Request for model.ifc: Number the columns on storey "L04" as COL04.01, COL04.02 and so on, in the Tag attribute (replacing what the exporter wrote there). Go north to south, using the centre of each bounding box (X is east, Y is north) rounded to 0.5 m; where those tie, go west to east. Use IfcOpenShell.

First a look at what the model holds.

```python
import ifcopenshell
import ifcopenshell.util.element
import ifcopenshell.util.placement

model = ifcopenshell.open("model.ifc")
print(model.schema)
storey = next(s for s in model.by_type("IfcBuildingStorey") if s.Name == "L04")
columns = [e for e in ifcopenshell.util.element.get_decomposition(storey) if e.is_a("IfcColumn")]
for e in sorted(columns, key=lambda e: e.id()):
    origin = ifcopenshell.util.placement.get_local_placement(e.ObjectPlacement)[:3, 3]
    print(e.id(), e.Tag, e.Name, origin.round(2) + 0.0, sep=" | ")
```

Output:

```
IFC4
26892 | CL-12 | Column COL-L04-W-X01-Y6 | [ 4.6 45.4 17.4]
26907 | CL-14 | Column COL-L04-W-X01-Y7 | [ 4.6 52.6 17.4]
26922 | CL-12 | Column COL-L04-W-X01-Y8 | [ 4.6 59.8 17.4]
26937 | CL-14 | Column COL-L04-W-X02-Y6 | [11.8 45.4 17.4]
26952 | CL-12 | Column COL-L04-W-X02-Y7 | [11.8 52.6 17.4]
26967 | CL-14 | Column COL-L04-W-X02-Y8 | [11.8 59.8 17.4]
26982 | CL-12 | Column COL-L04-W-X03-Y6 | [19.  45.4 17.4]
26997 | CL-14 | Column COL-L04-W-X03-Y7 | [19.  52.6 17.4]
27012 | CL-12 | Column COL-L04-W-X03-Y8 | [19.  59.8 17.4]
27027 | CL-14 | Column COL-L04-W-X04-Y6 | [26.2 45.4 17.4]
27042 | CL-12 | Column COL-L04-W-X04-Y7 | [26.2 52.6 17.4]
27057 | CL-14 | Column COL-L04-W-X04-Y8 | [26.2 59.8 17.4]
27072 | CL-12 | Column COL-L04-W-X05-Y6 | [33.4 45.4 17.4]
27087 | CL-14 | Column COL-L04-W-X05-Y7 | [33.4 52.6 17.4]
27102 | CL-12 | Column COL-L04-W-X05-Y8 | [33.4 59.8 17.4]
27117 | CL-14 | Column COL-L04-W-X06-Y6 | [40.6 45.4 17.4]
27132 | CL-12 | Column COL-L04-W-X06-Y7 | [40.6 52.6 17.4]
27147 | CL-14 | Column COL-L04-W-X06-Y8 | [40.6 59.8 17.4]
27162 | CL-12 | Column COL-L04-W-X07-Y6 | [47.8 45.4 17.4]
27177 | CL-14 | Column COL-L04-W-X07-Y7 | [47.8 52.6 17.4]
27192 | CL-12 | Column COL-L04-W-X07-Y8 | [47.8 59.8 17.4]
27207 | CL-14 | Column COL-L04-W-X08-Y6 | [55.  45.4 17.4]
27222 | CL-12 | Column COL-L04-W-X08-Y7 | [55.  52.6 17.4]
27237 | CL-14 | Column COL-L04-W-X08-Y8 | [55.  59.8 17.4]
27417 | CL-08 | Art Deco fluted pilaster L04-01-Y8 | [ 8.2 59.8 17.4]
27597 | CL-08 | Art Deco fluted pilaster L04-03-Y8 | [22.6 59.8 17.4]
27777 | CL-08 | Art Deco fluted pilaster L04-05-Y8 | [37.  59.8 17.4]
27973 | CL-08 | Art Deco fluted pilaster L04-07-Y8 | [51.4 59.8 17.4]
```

```python
import ifcopenshell
import ifcopenshell.geom
import ifcopenshell.util.element
import ifcopenshell.util.shape

model = ifcopenshell.open("model.ifc")
settings = ifcopenshell.geom.settings()
settings.set("use-world-coords", True)


def centre(element):
    shape = ifcopenshell.geom.create_shape(settings, element)
    return ifcopenshell.util.shape.get_bbox_centroid(shape.geometry)


storey = next(s for s in model.by_type("IfcBuildingStorey") if s.Name == "L04")
columns = [e for e in ifcopenshell.util.element.get_decomposition(storey) if e.is_a("IfcColumn")]

# Insertion points can sit at a corner or the storey origin, so sort by the geometry (in metres).
centres = {e: centre(e) for e in columns}
columns.sort(key=lambda e: (-round(centres[e][1] / 0.5), centres[e][0]))

for i, e in enumerate(columns, start=1):
    number = f"COL04.{i:02d}"
    e.Tag = number
    print(e.id(), number)

model.write("model_rev.ifc")
```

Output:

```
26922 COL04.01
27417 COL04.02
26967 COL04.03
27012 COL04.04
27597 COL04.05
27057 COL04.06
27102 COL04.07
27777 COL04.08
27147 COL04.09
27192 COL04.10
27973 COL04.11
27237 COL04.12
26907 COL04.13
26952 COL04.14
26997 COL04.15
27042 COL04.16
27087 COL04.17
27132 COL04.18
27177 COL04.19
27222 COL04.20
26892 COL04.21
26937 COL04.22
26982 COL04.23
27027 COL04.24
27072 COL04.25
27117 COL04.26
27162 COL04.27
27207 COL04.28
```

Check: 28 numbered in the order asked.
